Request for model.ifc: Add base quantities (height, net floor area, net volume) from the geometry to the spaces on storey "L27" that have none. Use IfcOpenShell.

First a look at what the model holds.

```python
import ifcopenshell
import ifcopenshell.util.element
import ifcopenshell.util.unit

model = ifcopenshell.open("model.ifc")
print(model.schema)
for unit_type in ("LENGTHUNIT", "AREAUNIT", "VOLUMEUNIT"):
    print(unit_type, ifcopenshell.util.unit.calculate_unit_scale(model, unit_type))
storey = next(s for s in model.by_type("IfcBuildingStorey") if s.Name == "L27")
spaces = [e for e in ifcopenshell.util.element.get_decomposition(storey) if e.is_a("IfcSpace")]
for e in sorted(spaces, key=lambda e: e.id()):
    print(e.id(), e.is_a(), e.Name, list(ifcopenshell.util.element.get_psets(e, qtos_only=True)), sep=" | ")
```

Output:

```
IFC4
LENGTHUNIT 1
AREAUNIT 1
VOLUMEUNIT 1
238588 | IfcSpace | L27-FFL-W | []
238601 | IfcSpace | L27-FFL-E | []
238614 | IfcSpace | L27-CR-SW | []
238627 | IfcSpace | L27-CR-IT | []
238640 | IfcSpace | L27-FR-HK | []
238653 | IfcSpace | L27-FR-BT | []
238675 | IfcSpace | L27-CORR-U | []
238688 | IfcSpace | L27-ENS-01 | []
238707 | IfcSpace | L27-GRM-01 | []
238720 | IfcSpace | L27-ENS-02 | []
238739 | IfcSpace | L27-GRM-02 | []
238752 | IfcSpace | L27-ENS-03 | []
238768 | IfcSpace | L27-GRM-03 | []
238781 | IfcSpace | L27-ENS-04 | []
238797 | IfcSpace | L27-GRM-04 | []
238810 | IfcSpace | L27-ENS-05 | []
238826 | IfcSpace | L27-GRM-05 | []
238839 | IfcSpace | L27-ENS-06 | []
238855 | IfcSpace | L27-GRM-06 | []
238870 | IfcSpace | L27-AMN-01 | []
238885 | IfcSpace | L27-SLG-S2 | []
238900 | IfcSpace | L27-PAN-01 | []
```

```python
import ifcopenshell
import ifcopenshell.api.pset
import ifcopenshell.geom
import ifcopenshell.util.element
import ifcopenshell.util.shape
import ifcopenshell.util.unit

model = ifcopenshell.open("model.ifc")
unit_scale = ifcopenshell.util.unit.calculate_unit_scale(model)
area_scale = ifcopenshell.util.unit.calculate_unit_scale(model, "AREAUNIT")
volume_scale = ifcopenshell.util.unit.calculate_unit_scale(model, "VOLUMEUNIT")
settings = ifcopenshell.geom.settings()

storey = next(s for s in model.by_type("IfcBuildingStorey") if s.Name == "L27")
spaces = [e for e in ifcopenshell.util.element.get_decomposition(storey) if e.is_a("IfcSpace")]

for e in sorted(spaces, key=lambda e: e.id()):
    if ifcopenshell.util.element.get_psets(e, qtos_only=True, should_inherit=False):
        continue
    # Geometry comes back in metres, in the element's own axes.
    shape = ifcopenshell.geom.create_shape(settings, e)
    values = {
        "Height": ifcopenshell.util.shape.get_z(shape.geometry) / unit_scale,
        "NetFloorArea": ifcopenshell.util.shape.get_footprint_area(shape.geometry) / area_scale,
        "NetVolume": ifcopenshell.util.shape.get_volume(shape.geometry) / volume_scale,
    }
    qto = ifcopenshell.api.pset.add_qto(model, product=e, name="Qto_SpaceBaseQuantities")
    ifcopenshell.api.pset.edit_qto(model, qto=qto, properties=values)
    print(e.id(), {k: round(v, 3) for k, v in values.items()})

model.write("model_rev.ifc")
```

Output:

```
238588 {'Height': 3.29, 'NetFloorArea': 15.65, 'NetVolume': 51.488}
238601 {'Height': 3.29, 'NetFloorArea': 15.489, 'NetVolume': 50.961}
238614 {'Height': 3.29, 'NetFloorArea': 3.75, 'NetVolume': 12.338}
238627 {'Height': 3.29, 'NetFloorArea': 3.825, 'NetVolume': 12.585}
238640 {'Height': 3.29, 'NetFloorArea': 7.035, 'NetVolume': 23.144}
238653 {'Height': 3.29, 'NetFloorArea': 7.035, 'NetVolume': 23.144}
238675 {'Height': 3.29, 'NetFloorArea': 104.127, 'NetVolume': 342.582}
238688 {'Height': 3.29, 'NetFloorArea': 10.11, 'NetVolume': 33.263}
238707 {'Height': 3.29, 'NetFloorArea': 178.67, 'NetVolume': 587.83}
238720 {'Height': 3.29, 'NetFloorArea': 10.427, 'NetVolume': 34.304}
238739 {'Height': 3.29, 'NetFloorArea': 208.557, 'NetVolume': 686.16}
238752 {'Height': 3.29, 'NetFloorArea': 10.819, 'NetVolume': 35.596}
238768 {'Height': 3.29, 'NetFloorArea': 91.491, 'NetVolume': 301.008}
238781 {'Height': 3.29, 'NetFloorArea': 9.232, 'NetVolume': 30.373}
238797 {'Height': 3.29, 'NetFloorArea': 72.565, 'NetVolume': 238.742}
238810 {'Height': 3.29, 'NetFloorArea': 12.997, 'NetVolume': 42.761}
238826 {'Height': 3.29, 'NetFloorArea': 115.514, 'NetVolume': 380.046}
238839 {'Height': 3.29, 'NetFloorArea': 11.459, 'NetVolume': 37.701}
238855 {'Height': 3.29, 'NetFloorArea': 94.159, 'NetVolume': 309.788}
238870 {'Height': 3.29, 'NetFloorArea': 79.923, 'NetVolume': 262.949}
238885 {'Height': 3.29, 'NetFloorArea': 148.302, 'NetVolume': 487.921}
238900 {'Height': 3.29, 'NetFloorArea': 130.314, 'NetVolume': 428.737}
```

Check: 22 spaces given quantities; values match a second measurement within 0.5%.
